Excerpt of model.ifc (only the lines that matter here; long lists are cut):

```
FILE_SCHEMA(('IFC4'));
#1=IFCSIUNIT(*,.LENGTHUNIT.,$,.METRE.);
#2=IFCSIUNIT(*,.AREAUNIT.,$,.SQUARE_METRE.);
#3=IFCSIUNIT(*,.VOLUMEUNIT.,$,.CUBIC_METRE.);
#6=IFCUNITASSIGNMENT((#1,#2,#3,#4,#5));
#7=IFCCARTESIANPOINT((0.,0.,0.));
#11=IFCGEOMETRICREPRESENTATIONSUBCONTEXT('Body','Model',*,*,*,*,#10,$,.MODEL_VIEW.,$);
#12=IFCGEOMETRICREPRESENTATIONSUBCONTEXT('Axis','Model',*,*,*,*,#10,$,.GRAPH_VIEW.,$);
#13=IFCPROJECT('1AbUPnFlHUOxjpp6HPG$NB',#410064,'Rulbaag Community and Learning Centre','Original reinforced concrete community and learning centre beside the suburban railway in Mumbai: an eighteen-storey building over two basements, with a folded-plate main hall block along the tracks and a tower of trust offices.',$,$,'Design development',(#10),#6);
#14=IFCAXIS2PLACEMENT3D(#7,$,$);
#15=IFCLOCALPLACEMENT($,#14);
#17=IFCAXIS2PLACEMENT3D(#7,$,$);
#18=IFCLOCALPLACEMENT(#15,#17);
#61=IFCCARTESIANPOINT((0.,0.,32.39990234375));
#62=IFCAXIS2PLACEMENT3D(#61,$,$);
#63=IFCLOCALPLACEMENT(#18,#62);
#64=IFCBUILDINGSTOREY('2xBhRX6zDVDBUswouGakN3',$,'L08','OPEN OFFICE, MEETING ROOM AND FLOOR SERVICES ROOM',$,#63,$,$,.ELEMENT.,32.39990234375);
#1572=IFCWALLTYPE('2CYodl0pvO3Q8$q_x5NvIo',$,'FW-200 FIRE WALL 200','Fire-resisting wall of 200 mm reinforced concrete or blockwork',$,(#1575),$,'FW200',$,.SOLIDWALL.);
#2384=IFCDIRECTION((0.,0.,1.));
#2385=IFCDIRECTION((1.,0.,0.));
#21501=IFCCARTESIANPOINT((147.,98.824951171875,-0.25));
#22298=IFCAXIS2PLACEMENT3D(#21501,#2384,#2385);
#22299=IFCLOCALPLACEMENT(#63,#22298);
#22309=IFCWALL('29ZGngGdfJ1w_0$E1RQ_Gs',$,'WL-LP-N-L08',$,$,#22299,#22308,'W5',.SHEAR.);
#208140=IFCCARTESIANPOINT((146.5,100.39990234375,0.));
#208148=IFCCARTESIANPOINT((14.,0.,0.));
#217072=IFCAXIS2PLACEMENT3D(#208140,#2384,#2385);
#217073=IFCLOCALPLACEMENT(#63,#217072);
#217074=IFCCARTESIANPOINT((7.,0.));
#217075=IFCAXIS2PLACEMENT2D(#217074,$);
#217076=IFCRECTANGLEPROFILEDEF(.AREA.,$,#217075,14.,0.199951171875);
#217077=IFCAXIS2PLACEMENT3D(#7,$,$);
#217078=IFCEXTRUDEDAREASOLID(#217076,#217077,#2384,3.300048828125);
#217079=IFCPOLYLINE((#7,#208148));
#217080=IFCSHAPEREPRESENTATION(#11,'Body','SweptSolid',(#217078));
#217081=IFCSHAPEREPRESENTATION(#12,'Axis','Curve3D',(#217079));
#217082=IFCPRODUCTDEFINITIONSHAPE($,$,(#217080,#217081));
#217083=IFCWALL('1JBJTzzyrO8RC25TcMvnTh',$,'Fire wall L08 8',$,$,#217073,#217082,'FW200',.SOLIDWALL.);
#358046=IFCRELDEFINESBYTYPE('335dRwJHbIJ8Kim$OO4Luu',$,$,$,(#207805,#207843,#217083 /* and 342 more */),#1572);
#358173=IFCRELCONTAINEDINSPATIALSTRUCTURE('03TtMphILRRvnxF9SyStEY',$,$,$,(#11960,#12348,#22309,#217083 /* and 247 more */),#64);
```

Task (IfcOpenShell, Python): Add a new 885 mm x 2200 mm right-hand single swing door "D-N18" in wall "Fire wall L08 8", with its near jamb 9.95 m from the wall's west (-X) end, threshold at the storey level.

```python
import numpy as np
import ifcopenshell
import ifcopenshell.api.feature
import ifcopenshell.api.geometry
import ifcopenshell.api.root
import ifcopenshell.api.spatial
import ifcopenshell.geom
import ifcopenshell.util.element
import ifcopenshell.util.placement
import ifcopenshell.util.representation
import ifcopenshell.util.shape
import ifcopenshell.util.unit

model = ifcopenshell.open("model.ifc")
unit_scale = ifcopenshell.util.unit.calculate_unit_scale(model)
settings = ifcopenshell.geom.settings()


def volume(element):
    """Net volume in cubic metres, openings subtracted."""
    shape = ifcopenshell.geom.create_shape(settings, element)
    return ifcopenshell.util.shape.get_volume(shape.geometry)


wall = model.by_guid("1JBJTzzyrO8RC25TcMvnTh")
storey = ifcopenshell.util.element.get_container(wall, ifc_class="IfcBuildingStorey")
context = ifcopenshell.util.representation.get_context(model, "Model", "Body", "MODEL_VIEW")
before = volume(wall)

width, height, from_end, sill = 0.885, 2.2, 9.95, 0.0  # metres

# The wall runs along its own X axis, and the end named is its -X end.
wall_shape = ifcopenshell.geom.create_shape(settings, wall)
x, y, z = ifcopenshell.util.shape.get_vertices(wall_shape.geometry).T
start = x.min() + from_end
face, thickness = float(y.min()), float(y.max() - y.min())
wall_matrix = ifcopenshell.util.placement.get_local_placement(wall.ObjectPlacement)
level = ifcopenshell.util.placement.get_local_placement(storey.ObjectPlacement)[2, 3]


def in_wall(x, y):
    """Placement at x, y metres in the wall's axes, at sill height."""
    matrix = wall_matrix.copy()
    matrix[:, 3] = wall_matrix @ np.array([x / unit_scale, y / unit_scale, 0.0, 1.0])
    matrix[2, 3] = level + sill / unit_scale
    return matrix


# Opening: a box that overshoots both wall faces by 50 mm.
opening = ifcopenshell.api.root.create_entity(model, ifc_class="IfcOpeningElement", predefined_type="OPENING")
box = ifcopenshell.api.geometry.add_wall_representation(
    model, context=context, length=width, height=height, thickness=thickness + 0.1
)
ifcopenshell.api.geometry.assign_representation(model, product=opening, representation=box)
ifcopenshell.api.geometry.edit_object_placement(model, product=opening, matrix=in_wall(start, face - 0.05), is_si=False)
ifcopenshell.api.feature.add_feature(model, feature=opening, element=wall)

door = ifcopenshell.api.root.create_entity(model, ifc_class="IfcDoor", name="D-N18", predefined_type="DOOR")
door.OverallWidth, door.OverallHeight = width / unit_scale, height / unit_scale
door.OperationType = "SINGLE_SWING_RIGHT"
body = ifcopenshell.api.geometry.add_door_representation(
    model,
    context=context,
    overall_width=door.OverallWidth,
    overall_height=door.OverallHeight,
    operation_type="SINGLE_SWING_RIGHT",
    lining_properties={"LiningDepth": thickness / unit_scale, "ThresholdDepth": thickness / unit_scale},
)
ifcopenshell.api.geometry.assign_representation(model, product=door, representation=body)
ifcopenshell.api.spatial.assign_container(model, products=[door], relating_structure=storey)
ifcopenshell.api.feature.add_filling(model, opening=opening, element=door)

# The lining spans the wall, so the door starts at the wall face.
ifcopenshell.api.geometry.edit_object_placement(model, product=door, matrix=in_wall(start, face), is_si=False)

after = volume(wall)

print(f"wall volume {before:.3f} -> {after:.3f} m3")

model.write("model_updated.ifc")
```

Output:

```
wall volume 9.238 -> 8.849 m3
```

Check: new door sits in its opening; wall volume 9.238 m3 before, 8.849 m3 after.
